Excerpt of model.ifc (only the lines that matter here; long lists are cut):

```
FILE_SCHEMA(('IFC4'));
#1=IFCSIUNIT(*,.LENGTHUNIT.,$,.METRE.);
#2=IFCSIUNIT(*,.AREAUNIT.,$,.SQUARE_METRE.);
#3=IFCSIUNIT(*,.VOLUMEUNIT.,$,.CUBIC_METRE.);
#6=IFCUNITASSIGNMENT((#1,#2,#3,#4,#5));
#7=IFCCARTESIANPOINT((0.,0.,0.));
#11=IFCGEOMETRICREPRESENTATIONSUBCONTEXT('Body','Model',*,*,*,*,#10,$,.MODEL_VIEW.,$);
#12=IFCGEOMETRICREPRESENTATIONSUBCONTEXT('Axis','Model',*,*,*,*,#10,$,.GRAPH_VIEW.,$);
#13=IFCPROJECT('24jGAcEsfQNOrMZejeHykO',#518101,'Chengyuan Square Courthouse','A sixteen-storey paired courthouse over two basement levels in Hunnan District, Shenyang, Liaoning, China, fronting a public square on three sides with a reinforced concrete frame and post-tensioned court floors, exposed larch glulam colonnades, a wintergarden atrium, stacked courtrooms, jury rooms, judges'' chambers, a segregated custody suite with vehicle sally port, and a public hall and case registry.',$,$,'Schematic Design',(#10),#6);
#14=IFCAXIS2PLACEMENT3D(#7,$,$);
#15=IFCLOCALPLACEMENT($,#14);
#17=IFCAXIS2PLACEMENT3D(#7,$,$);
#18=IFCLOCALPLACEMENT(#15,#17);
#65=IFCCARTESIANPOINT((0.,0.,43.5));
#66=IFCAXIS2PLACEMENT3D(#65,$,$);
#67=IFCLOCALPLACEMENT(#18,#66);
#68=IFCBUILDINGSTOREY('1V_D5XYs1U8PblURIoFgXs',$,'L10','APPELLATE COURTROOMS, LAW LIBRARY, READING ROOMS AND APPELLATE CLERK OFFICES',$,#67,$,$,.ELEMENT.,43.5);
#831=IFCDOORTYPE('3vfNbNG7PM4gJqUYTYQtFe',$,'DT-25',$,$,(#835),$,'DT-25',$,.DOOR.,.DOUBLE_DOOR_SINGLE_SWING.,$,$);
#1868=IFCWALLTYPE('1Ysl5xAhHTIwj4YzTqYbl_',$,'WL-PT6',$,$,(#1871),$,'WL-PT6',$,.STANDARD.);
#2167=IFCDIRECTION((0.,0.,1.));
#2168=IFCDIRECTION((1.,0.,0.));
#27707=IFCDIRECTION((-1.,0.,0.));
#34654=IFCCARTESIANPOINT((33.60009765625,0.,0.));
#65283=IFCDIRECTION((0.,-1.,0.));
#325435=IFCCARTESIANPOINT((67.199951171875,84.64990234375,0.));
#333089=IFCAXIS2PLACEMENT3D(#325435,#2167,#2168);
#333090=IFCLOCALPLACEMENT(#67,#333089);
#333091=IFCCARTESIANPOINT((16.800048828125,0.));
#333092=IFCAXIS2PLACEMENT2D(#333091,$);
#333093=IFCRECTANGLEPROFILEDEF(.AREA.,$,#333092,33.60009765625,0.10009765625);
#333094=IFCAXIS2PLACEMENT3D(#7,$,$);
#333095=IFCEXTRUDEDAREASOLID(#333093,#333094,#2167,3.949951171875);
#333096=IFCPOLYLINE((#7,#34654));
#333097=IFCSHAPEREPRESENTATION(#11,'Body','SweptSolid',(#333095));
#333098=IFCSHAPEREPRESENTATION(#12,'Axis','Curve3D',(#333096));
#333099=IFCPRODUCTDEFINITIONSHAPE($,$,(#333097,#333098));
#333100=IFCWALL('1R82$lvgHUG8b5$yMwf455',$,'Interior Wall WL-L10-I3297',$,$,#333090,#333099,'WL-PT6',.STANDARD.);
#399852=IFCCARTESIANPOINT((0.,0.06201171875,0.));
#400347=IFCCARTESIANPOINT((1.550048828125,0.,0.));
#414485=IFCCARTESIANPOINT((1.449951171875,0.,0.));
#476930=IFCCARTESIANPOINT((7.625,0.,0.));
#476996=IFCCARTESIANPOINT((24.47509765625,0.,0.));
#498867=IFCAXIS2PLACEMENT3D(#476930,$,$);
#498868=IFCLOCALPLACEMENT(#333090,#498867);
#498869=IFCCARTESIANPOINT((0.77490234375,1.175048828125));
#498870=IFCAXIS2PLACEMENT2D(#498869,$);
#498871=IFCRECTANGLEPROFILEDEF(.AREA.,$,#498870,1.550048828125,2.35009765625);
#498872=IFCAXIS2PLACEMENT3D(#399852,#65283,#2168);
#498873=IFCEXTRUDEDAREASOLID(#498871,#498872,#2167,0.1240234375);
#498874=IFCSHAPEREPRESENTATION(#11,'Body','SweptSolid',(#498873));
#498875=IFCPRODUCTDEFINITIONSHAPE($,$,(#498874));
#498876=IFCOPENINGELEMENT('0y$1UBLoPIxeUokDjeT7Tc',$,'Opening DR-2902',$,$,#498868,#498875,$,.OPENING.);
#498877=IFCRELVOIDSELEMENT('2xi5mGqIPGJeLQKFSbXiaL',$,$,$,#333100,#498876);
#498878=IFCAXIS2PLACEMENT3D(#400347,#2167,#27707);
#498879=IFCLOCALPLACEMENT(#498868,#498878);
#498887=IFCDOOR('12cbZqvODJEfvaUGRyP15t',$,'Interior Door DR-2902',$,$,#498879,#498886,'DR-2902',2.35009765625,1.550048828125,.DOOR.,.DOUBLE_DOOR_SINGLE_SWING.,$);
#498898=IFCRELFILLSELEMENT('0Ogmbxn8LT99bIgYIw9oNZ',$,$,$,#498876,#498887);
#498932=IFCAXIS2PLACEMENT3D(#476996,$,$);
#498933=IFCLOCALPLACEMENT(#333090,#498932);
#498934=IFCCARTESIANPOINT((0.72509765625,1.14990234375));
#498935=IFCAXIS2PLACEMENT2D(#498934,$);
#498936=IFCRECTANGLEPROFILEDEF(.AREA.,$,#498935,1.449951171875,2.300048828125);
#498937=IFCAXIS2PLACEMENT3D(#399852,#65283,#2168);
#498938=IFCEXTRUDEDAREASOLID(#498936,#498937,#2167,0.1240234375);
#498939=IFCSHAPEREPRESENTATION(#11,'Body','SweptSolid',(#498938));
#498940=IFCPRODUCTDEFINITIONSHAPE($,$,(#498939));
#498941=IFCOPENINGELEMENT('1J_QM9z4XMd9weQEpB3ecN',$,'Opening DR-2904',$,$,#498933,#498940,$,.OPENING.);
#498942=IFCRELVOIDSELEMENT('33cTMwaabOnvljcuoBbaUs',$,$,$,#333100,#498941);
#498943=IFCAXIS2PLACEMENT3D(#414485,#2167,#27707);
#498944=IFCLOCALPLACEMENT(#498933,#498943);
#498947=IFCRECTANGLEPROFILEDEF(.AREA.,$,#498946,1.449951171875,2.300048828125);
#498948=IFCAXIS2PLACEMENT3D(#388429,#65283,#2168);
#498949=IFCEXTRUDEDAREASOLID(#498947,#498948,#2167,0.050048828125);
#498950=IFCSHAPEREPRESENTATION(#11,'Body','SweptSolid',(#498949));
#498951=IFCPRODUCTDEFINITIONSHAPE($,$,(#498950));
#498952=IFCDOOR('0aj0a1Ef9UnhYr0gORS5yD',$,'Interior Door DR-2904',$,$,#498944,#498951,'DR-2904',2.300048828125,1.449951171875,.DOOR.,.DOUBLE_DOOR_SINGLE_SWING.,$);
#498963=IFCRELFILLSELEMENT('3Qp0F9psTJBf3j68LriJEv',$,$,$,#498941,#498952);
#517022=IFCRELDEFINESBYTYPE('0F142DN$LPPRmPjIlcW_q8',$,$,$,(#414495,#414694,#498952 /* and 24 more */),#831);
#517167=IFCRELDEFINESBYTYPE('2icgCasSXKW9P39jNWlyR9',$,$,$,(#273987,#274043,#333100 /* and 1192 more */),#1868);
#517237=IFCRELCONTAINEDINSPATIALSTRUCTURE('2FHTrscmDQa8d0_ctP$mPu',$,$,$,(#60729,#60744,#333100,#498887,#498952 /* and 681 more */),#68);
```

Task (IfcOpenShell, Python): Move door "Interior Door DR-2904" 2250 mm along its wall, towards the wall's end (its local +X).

```python
import ifcopenshell
import ifcopenshell.api.geometry
import ifcopenshell.util.placement
import ifcopenshell.util.unit

model = ifcopenshell.open("model.ifc")
unit_scale = ifcopenshell.util.unit.calculate_unit_scale(model)

door = model.by_guid("0aj0a1Ef9UnhYr0gORS5yD")
opening = door.FillsVoids[0].RelatingOpeningElement
wall = opening.VoidsElements[0].RelatingBuildingElement

wall_matrix = ifcopenshell.util.placement.get_local_placement(wall.ObjectPlacement)
shift = wall_matrix[:3, 0] * 2.25 / unit_scale
before = ifcopenshell.util.placement.get_local_placement(door.ObjectPlacement)[:3, 3].copy()

# The door is placed relative to its opening, so it follows when the opening moves.
matrix = ifcopenshell.util.placement.get_local_placement(opening.ObjectPlacement)
matrix[:3, 3] += shift
ifcopenshell.api.geometry.edit_object_placement(
    model, product=opening, matrix=matrix, is_si=False, should_transform_children=True
)

after = ifcopenshell.util.placement.get_local_placement(door.ObjectPlacement)[:3, 3]
print("door moved by", (after - before).round(3) + 0.0)

model.write("model_updated.ifc")
```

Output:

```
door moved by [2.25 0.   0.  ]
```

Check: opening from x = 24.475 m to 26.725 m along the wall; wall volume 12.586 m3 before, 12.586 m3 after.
